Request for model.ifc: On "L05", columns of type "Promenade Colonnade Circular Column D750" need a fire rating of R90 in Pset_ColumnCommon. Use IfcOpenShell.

First a look at what the model holds.

```python
import ifcopenshell
import ifcopenshell.util.element

model = ifcopenshell.open("model.ifc")
print(model.schema)
storey = next(s for s in model.by_type("IfcBuildingStorey") if s.Name == "L05")
columns = [e for e in ifcopenshell.util.element.get_decomposition(storey) if e.is_a("IfcColumn")]
seen = {}
for e in columns:
    element_type = ifcopenshell.util.element.get_type(e)
    key = (element_type.Name if element_type != e and element_type else None, ifcopenshell.util.element.get_pset(e, "Pset_ColumnCommon", "FireRating"))
    seen[key] = seen.get(key, 0) + 1
for (name, value), count in sorted(seen.items(), key=str):
    print(count, "x", name, "|", value)
```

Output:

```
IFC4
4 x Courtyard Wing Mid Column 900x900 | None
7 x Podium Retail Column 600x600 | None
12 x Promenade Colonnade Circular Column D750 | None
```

```python
import ifcopenshell
import ifcopenshell.api.pset
import ifcopenshell.util.element

model = ifcopenshell.open("model.ifc")

storey = next(s for s in model.by_type("IfcBuildingStorey") if s.Name == "L05")
columns = [e for e in ifcopenshell.util.element.get_decomposition(storey) if e.is_a("IfcColumn")]

count = 0
for e in columns:
    element_type = ifcopenshell.util.element.get_type(e)
    if element_type in (None, e) or element_type.Name != "Promenade Colonnade Circular Column D750":
        continue
    # add_pset returns the element's existing set when there is one.
    pset = ifcopenshell.api.pset.add_pset(model, product=e, name="Pset_ColumnCommon")
    ifcopenshell.api.pset.edit_pset(model, pset=pset, properties={"FireRating": "R90"})
    count += 1

print(count, "columns updated")

model.write("model_edited.ifc")
```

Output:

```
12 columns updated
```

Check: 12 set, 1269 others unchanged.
